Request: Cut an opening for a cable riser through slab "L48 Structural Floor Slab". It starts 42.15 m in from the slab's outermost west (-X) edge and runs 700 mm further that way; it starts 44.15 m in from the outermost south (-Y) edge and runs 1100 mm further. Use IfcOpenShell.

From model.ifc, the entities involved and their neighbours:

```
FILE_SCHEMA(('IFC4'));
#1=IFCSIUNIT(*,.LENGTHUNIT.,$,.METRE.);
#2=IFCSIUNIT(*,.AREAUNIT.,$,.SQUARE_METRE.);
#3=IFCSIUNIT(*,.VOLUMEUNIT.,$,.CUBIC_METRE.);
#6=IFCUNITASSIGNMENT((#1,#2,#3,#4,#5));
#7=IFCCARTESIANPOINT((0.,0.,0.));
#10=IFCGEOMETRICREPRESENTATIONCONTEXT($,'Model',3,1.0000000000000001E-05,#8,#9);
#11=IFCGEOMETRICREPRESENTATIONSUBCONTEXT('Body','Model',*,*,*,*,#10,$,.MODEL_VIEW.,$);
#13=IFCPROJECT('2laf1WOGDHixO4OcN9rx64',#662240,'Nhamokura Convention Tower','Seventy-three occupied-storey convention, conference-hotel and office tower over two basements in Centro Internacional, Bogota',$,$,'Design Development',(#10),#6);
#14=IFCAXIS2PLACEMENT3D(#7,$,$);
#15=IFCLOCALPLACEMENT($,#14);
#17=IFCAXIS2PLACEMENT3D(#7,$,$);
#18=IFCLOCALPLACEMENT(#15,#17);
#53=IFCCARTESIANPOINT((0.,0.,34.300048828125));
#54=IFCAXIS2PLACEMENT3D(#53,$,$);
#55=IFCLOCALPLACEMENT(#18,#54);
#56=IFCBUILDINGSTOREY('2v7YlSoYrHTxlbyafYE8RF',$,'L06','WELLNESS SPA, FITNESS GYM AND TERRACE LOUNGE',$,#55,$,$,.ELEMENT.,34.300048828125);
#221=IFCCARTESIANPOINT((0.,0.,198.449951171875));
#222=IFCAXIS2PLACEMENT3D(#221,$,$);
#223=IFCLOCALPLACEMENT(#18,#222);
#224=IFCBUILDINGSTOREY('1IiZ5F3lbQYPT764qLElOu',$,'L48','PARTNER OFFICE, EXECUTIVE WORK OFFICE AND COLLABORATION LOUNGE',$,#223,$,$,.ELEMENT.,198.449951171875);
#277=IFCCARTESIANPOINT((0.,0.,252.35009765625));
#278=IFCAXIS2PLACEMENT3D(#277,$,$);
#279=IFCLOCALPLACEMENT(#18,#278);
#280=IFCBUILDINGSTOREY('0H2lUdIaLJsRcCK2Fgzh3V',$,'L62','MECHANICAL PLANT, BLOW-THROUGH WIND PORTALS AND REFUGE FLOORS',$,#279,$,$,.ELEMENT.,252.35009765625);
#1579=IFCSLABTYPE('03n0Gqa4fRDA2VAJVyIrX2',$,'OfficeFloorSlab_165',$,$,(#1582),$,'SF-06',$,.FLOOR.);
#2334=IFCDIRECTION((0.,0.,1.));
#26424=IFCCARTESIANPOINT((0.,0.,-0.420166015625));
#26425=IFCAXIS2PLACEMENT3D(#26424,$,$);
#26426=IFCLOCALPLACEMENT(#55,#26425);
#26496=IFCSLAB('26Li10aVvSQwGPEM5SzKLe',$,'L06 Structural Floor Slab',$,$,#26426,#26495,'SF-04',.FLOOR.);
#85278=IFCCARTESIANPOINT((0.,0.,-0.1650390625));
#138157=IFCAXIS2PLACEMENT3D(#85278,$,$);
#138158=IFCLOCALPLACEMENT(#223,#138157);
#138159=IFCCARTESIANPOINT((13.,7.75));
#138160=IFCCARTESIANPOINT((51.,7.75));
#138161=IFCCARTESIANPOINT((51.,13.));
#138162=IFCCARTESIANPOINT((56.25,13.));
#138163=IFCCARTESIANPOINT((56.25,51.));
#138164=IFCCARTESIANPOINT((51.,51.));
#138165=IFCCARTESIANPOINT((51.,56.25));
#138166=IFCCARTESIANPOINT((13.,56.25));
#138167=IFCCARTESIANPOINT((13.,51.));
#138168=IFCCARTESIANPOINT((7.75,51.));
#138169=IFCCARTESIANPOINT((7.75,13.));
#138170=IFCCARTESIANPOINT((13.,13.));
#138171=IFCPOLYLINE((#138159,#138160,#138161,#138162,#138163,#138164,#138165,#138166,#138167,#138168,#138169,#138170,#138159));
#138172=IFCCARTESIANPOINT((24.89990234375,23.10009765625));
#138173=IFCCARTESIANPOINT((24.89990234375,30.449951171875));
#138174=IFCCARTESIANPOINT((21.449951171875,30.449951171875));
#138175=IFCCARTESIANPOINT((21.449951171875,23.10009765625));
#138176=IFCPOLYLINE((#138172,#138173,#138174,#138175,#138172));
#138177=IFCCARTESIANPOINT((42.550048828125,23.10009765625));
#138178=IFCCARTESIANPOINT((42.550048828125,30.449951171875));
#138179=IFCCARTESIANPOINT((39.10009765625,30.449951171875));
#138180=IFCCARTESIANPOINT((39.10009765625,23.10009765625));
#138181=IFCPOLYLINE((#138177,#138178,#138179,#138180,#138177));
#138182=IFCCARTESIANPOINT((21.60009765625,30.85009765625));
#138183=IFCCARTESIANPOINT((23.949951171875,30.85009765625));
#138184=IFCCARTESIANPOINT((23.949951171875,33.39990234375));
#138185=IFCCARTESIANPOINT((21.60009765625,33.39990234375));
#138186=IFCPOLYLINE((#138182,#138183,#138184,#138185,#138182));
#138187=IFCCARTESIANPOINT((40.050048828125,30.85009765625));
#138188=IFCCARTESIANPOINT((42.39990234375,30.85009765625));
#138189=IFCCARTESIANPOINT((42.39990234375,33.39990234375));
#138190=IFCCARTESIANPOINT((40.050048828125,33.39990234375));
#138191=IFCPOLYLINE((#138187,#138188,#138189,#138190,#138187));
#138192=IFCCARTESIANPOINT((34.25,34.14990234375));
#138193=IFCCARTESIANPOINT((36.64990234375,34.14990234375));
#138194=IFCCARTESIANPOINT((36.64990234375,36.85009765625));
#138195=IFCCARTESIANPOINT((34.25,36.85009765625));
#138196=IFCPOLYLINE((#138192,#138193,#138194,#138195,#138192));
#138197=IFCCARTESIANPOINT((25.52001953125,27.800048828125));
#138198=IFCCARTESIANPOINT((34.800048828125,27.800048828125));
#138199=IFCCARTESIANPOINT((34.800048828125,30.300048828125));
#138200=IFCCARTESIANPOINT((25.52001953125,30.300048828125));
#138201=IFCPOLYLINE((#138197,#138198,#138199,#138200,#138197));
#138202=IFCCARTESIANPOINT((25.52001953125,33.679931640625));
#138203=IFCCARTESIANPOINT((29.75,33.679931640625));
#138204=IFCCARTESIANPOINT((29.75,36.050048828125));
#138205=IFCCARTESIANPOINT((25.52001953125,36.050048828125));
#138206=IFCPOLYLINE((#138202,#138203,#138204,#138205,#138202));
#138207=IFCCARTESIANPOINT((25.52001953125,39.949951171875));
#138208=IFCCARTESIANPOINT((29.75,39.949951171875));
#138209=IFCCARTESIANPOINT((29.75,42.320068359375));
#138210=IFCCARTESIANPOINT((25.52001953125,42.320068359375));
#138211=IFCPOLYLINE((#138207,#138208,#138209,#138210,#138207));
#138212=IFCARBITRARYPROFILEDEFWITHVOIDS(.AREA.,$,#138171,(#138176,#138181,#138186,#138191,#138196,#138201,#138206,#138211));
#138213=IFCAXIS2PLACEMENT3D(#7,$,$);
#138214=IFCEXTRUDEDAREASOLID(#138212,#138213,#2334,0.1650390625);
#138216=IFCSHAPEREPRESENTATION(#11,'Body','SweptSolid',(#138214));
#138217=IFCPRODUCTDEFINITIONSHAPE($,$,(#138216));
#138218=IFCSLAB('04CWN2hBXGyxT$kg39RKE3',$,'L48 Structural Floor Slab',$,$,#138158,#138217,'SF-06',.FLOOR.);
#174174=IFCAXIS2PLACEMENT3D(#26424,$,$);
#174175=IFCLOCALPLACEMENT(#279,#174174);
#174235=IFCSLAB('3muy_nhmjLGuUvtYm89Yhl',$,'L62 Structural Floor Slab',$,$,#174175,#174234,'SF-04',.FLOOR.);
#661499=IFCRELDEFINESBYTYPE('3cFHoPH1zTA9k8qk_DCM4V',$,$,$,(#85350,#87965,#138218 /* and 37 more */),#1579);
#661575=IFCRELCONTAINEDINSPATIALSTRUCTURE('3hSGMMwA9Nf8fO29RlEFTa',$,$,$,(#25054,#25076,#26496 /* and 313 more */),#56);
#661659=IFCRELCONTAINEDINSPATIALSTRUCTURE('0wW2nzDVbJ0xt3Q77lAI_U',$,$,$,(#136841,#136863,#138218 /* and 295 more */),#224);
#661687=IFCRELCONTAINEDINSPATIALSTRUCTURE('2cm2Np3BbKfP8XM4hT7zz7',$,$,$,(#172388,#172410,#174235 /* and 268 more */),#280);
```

```python
import numpy as np
import ifcopenshell
import ifcopenshell.api.feature
import ifcopenshell.api.geometry
import ifcopenshell.api.root
import ifcopenshell.geom
import ifcopenshell.util.placement
import ifcopenshell.util.representation
import ifcopenshell.util.shape
import ifcopenshell.util.unit

model = ifcopenshell.open("model.ifc")
unit_scale = ifcopenshell.util.unit.calculate_unit_scale(model)
settings = ifcopenshell.geom.settings()


def volume(element):
    """Net volume in cubic metres, openings subtracted."""
    shape = ifcopenshell.geom.create_shape(settings, element)
    return ifcopenshell.util.shape.get_volume(shape.geometry)


slab = model.by_guid("04CWN2hBXGyxT$kg39RKE3")
before = volume(slab)

# Extent in the slab's own axes, in metres. The edges named are its -X and -Y sides.
slab_shape = ifcopenshell.geom.create_shape(settings, slab)
vertices = ifcopenshell.util.shape.get_vertices(slab_shape.geometry)
x_min, y_min, bottom = vertices.min(axis=0)
top = vertices[:, 2].max()

opening = ifcopenshell.api.root.create_entity(model, ifc_class="IfcOpeningElement", name="Cable riser opening", predefined_type="OPENING")
context = ifcopenshell.util.representation.get_context(model, "Model", "Body", "MODEL_VIEW")
width, depth = 0.7, 1.1
outline = [(0.0, 0.0), (width, 0.0), (width, depth), (0.0, depth), (0.0, 0.0)]
# Overshoot both faces by 50 mm so the cut is clean.
shape = ifcopenshell.api.geometry.add_slab_representation(
    model, context=context, depth=top - bottom + 0.1, polyline=outline
)
ifcopenshell.api.geometry.assign_representation(model, product=opening, representation=shape)

matrix = ifcopenshell.util.placement.get_local_placement(slab.ObjectPlacement)
matrix[:, 3] = matrix @ np.append(np.array([x_min + 42.15, y_min + 44.15, bottom - 0.05]) / unit_scale, 1.0)
ifcopenshell.api.geometry.edit_object_placement(model, product=opening, matrix=matrix, is_si=False)
ifcopenshell.api.feature.add_feature(model, feature=opening, element=slab)

after = volume(slab)

print(f"slab volume {before:.3f} -> {after:.3f} m3")

model.write("model_rev.ifc")
```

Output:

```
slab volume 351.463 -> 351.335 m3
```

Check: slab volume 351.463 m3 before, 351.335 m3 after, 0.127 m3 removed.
